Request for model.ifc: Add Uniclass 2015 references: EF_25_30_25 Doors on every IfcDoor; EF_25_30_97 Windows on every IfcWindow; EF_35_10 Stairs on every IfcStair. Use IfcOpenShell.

First a look at what the model holds.

```python
import ifcopenshell

model = ifcopenshell.open("model.ifc")
print(model.schema)
print("classifications:", [c.Name for c in model.by_type("IfcClassification")])
for ifc_class in ("IfcDoor", "IfcRoof", "IfcStair", "IfcWall", "IfcWindow"):
    print(ifc_class, len(model.by_type(ifc_class)))
```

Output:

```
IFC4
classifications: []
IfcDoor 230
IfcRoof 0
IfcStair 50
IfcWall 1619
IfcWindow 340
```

```python
import ifcopenshell
import ifcopenshell.api.classification

model = ifcopenshell.open("model.ifc")

system = ifcopenshell.api.classification.add_classification(model, classification="Uniclass 2015")

codes = {
    "IfcDoor": ("EF_25_30_25", "Doors"),
    "IfcWindow": ("EF_25_30_97", "Windows"),
    "IfcStair": ("EF_35_10", "Stairs"),
}
for ifc_class, (code, name) in codes.items():
    products = model.by_type(ifc_class)
    ifcopenshell.api.classification.add_reference(
        model, products=products, classification=system, identification=code, name=name
    )
    print(code, len(products))

model.write("model_updated.ifc")
```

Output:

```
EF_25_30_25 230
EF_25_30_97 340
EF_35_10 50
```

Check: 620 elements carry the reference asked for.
